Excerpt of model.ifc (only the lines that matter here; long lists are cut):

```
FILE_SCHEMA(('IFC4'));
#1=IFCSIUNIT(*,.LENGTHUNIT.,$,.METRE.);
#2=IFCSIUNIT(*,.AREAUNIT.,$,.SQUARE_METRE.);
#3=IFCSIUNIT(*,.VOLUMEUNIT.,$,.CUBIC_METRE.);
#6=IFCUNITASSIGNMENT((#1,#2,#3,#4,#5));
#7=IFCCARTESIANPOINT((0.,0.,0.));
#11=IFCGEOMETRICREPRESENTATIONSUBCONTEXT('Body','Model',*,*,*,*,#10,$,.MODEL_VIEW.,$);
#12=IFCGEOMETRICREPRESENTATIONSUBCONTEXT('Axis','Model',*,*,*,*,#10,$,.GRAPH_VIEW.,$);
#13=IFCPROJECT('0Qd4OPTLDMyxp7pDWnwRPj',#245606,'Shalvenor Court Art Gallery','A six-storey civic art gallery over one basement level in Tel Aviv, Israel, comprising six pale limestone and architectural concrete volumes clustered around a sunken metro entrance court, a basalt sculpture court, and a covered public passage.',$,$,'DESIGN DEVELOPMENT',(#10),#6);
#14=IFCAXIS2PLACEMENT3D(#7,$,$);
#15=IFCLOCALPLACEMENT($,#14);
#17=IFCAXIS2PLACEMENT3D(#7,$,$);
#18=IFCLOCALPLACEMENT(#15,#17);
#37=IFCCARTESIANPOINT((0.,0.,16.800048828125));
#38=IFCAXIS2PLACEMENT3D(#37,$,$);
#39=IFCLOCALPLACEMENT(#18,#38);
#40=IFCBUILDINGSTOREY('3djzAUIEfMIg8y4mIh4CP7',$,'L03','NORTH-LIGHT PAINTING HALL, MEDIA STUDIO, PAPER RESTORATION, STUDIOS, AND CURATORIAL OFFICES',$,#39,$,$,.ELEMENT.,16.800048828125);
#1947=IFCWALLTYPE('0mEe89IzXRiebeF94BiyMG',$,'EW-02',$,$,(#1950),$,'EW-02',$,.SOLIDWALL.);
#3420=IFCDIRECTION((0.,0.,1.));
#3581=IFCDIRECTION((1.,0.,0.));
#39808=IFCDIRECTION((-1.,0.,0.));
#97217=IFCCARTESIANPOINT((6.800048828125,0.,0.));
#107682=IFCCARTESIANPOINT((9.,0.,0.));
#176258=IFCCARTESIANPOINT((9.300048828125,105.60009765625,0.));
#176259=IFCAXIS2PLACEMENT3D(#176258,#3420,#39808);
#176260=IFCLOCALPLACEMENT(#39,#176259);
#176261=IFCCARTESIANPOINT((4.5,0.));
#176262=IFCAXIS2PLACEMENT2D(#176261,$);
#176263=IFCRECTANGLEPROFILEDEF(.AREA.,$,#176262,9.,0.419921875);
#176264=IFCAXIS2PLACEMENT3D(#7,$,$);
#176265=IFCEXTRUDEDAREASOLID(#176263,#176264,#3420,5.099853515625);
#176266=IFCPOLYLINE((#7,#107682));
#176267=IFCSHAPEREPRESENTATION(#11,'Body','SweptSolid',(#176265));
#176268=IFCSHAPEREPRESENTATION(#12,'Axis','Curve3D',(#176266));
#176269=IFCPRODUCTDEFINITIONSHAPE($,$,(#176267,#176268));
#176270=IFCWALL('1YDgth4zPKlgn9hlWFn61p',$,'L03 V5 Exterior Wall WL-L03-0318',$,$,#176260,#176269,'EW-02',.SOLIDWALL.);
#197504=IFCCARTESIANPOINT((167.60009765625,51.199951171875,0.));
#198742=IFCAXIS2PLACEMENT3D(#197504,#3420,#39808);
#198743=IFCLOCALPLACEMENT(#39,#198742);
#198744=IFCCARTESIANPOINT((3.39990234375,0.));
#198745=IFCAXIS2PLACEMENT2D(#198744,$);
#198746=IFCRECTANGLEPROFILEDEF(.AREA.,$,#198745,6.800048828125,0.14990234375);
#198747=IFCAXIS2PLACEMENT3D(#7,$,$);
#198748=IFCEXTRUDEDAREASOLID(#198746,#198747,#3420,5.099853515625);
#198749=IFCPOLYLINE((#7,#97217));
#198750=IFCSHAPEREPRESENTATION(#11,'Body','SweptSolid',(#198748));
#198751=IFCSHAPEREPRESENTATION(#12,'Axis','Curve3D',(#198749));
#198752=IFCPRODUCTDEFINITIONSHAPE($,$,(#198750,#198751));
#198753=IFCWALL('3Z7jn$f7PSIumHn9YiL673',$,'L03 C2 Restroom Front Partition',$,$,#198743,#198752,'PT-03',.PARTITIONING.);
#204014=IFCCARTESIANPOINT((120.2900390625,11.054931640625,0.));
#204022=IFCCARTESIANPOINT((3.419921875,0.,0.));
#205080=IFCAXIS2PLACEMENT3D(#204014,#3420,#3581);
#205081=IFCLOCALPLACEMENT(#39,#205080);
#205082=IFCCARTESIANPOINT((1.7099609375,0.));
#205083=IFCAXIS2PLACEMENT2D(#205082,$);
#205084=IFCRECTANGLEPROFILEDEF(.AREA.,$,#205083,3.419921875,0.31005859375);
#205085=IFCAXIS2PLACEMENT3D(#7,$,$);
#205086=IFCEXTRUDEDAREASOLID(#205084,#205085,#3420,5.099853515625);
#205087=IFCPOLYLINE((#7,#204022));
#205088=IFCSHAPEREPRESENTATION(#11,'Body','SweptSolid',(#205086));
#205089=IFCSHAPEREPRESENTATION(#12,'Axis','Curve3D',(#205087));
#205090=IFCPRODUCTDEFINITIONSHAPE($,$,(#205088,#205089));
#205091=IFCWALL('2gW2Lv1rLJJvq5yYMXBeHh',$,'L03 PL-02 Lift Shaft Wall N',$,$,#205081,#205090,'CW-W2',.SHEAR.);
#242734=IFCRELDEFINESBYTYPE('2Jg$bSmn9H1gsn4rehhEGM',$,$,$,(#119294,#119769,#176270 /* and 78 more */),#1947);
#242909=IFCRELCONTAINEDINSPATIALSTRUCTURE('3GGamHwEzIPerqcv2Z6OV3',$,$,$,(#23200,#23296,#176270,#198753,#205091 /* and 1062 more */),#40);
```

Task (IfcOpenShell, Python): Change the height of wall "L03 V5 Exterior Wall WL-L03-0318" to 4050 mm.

```python
import ifcopenshell
import ifcopenshell.geom
import ifcopenshell.util.representation
import ifcopenshell.util.shape
import ifcopenshell.util.unit

model = ifcopenshell.open("model.ifc")
unit_scale = ifcopenshell.util.unit.calculate_unit_scale(model)
settings = ifcopenshell.geom.settings()


def volume(element):
    """Net volume in cubic metres, openings subtracted."""
    shape = ifcopenshell.geom.create_shape(settings, element)
    return ifcopenshell.util.shape.get_volume(shape.geometry)


wall = model.by_guid("1YDgth4zPKlgn9hlWFn61p")
before = volume(wall)

body = ifcopenshell.util.representation.get_representation(wall, "Model", "Body")
solid = body.Items[0]
old_height = solid.Depth
solid.Depth = 4.05 / unit_scale
after = volume(wall)

print(f"height {old_height:g} -> {solid.Depth:g}, volume {before:.3f} -> {after:.3f} m3")

model.write("model_rev.ifc")
```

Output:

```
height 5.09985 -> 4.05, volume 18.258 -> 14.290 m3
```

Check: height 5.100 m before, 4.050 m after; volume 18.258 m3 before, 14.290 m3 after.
